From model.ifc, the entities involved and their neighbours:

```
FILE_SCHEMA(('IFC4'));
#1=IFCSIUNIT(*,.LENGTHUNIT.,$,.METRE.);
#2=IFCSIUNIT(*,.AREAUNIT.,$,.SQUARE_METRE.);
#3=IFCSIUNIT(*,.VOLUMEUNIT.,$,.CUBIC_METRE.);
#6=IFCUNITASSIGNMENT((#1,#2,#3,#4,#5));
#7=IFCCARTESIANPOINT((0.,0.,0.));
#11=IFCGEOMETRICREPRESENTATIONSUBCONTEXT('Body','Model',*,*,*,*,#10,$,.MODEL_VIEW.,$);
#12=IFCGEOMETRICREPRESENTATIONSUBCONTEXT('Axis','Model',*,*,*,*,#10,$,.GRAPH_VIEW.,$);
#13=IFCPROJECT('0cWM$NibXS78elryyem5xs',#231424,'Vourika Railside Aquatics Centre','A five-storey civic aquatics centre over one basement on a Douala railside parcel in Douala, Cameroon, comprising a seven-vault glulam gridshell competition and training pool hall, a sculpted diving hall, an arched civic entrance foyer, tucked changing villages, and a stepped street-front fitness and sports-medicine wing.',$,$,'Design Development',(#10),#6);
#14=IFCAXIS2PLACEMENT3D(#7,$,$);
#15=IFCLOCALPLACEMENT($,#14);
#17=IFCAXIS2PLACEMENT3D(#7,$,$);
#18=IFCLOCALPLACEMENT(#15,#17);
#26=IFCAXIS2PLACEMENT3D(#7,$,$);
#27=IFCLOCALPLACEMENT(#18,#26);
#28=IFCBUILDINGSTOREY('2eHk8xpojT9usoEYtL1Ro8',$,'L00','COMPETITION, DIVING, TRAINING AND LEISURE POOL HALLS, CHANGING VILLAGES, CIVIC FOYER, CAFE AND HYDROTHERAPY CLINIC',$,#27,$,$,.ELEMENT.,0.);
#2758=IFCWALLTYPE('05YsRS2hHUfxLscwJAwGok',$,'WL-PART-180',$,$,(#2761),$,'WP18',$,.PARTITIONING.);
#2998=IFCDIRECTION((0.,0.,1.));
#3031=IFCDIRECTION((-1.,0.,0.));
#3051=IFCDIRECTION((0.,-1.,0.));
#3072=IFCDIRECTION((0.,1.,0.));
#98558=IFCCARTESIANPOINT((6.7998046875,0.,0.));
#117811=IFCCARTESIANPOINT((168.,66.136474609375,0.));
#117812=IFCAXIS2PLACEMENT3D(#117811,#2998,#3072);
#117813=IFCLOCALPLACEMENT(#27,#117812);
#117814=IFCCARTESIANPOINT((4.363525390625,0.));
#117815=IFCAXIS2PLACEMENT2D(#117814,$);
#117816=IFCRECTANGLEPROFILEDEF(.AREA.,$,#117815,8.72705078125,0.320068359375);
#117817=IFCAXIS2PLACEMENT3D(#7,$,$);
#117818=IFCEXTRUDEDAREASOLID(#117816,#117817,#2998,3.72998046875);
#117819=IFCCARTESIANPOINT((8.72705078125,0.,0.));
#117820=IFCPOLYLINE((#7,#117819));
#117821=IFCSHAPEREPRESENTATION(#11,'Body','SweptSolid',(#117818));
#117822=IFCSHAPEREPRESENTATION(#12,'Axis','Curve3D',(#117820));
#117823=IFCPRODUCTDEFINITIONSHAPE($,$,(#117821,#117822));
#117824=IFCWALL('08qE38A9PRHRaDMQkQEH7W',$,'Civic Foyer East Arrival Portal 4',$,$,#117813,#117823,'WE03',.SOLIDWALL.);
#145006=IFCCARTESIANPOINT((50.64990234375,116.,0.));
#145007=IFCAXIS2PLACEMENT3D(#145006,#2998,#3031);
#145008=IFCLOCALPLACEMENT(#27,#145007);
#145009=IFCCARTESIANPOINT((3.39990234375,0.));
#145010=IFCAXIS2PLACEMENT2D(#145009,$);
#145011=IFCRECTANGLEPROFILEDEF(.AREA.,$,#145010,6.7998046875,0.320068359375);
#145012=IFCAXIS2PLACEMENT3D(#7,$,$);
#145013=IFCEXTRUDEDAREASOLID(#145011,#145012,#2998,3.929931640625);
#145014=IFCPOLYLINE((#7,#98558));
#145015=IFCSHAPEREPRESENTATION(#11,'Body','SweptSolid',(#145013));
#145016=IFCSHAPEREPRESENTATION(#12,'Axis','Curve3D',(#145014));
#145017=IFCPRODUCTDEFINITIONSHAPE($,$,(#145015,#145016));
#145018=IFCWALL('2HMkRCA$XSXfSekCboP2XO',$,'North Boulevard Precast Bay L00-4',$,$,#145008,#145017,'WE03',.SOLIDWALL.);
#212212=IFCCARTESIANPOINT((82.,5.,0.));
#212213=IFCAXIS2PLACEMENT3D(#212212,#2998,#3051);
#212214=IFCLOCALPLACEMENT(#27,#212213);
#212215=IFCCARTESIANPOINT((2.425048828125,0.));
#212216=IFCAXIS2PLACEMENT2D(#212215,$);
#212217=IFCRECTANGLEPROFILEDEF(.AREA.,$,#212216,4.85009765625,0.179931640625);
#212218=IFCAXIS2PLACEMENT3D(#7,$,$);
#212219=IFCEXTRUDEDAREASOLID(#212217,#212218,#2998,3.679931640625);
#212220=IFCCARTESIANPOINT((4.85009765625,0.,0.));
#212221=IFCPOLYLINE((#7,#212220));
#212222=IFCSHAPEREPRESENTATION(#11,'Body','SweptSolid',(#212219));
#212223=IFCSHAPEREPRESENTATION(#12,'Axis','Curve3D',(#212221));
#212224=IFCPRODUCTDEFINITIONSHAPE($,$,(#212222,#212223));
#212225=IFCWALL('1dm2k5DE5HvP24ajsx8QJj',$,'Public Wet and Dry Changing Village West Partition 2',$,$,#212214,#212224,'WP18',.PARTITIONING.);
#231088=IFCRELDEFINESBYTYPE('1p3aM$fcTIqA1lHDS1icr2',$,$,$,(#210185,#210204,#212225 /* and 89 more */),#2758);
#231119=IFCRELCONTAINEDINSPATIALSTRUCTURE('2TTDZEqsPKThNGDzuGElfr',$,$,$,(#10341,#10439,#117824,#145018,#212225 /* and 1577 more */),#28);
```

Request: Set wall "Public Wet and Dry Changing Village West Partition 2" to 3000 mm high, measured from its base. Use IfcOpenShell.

```python
import ifcopenshell
import ifcopenshell.geom
import ifcopenshell.util.representation
import ifcopenshell.util.shape
import ifcopenshell.util.unit

model = ifcopenshell.open("model.ifc")
unit_scale = ifcopenshell.util.unit.calculate_unit_scale(model)
settings = ifcopenshell.geom.settings()


def volume(element):
    """Net volume in cubic metres, openings subtracted."""
    shape = ifcopenshell.geom.create_shape(settings, element)
    return ifcopenshell.util.shape.get_volume(shape.geometry)


wall = model.by_id(212225)
before = volume(wall)

body = ifcopenshell.util.representation.get_representation(wall, "Model", "Body")
solid = body.Items[0]
old_height = solid.Depth
solid.Depth = 3 / unit_scale
after = volume(wall)

print(f"height {old_height:g} -> {solid.Depth:g}, volume {before:.3f} -> {after:.3f} m3")

model.write("model_edited.ifc")
```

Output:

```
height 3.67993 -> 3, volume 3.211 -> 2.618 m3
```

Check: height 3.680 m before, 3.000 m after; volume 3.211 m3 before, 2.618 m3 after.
